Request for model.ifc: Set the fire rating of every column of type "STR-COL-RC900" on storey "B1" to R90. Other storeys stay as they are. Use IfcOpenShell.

First a look at what the model holds.

```python
import ifcopenshell
import ifcopenshell.util.element

model = ifcopenshell.open("model.ifc")
print(model.schema)
storey = next(s for s in model.by_type("IfcBuildingStorey") if s.Name == "B1")
columns = [e for e in ifcopenshell.util.element.get_decomposition(storey) if e.is_a("IfcColumn")]
seen = {}
for e in columns:
    element_type = ifcopenshell.util.element.get_type(e)
    key = (element_type.Name if element_type != e and element_type else None, ifcopenshell.util.element.get_pset(e, "Pset_ColumnCommon", "FireRating"))
    seen[key] = seen.get(key, 0) + 1
for (name, value), count in sorted(seen.items(), key=str):
    print(count, "x", name, "|", value)
```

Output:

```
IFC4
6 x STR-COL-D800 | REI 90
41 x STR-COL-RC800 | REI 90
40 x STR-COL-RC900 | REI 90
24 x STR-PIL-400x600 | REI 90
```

```python
import ifcopenshell
import ifcopenshell.api.pset
import ifcopenshell.util.element

model = ifcopenshell.open("model.ifc")

storey = next(s for s in model.by_type("IfcBuildingStorey") if s.Name == "B1")
columns = [e for e in ifcopenshell.util.element.get_decomposition(storey) if e.is_a("IfcColumn")]

count = 0
for e in columns:
    element_type = ifcopenshell.util.element.get_type(e)
    if element_type in (None, e) or element_type.Name != "STR-COL-RC900":
        continue
    # add_pset returns the element's existing set when there is one.
    pset = ifcopenshell.api.pset.add_pset(model, product=e, name="Pset_ColumnCommon")
    ifcopenshell.api.pset.edit_pset(model, pset=pset, properties={"FireRating": "R90"})
    count += 1

print(count, "columns updated")

model.write("model-out.ifc")
```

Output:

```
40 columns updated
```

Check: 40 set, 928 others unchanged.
